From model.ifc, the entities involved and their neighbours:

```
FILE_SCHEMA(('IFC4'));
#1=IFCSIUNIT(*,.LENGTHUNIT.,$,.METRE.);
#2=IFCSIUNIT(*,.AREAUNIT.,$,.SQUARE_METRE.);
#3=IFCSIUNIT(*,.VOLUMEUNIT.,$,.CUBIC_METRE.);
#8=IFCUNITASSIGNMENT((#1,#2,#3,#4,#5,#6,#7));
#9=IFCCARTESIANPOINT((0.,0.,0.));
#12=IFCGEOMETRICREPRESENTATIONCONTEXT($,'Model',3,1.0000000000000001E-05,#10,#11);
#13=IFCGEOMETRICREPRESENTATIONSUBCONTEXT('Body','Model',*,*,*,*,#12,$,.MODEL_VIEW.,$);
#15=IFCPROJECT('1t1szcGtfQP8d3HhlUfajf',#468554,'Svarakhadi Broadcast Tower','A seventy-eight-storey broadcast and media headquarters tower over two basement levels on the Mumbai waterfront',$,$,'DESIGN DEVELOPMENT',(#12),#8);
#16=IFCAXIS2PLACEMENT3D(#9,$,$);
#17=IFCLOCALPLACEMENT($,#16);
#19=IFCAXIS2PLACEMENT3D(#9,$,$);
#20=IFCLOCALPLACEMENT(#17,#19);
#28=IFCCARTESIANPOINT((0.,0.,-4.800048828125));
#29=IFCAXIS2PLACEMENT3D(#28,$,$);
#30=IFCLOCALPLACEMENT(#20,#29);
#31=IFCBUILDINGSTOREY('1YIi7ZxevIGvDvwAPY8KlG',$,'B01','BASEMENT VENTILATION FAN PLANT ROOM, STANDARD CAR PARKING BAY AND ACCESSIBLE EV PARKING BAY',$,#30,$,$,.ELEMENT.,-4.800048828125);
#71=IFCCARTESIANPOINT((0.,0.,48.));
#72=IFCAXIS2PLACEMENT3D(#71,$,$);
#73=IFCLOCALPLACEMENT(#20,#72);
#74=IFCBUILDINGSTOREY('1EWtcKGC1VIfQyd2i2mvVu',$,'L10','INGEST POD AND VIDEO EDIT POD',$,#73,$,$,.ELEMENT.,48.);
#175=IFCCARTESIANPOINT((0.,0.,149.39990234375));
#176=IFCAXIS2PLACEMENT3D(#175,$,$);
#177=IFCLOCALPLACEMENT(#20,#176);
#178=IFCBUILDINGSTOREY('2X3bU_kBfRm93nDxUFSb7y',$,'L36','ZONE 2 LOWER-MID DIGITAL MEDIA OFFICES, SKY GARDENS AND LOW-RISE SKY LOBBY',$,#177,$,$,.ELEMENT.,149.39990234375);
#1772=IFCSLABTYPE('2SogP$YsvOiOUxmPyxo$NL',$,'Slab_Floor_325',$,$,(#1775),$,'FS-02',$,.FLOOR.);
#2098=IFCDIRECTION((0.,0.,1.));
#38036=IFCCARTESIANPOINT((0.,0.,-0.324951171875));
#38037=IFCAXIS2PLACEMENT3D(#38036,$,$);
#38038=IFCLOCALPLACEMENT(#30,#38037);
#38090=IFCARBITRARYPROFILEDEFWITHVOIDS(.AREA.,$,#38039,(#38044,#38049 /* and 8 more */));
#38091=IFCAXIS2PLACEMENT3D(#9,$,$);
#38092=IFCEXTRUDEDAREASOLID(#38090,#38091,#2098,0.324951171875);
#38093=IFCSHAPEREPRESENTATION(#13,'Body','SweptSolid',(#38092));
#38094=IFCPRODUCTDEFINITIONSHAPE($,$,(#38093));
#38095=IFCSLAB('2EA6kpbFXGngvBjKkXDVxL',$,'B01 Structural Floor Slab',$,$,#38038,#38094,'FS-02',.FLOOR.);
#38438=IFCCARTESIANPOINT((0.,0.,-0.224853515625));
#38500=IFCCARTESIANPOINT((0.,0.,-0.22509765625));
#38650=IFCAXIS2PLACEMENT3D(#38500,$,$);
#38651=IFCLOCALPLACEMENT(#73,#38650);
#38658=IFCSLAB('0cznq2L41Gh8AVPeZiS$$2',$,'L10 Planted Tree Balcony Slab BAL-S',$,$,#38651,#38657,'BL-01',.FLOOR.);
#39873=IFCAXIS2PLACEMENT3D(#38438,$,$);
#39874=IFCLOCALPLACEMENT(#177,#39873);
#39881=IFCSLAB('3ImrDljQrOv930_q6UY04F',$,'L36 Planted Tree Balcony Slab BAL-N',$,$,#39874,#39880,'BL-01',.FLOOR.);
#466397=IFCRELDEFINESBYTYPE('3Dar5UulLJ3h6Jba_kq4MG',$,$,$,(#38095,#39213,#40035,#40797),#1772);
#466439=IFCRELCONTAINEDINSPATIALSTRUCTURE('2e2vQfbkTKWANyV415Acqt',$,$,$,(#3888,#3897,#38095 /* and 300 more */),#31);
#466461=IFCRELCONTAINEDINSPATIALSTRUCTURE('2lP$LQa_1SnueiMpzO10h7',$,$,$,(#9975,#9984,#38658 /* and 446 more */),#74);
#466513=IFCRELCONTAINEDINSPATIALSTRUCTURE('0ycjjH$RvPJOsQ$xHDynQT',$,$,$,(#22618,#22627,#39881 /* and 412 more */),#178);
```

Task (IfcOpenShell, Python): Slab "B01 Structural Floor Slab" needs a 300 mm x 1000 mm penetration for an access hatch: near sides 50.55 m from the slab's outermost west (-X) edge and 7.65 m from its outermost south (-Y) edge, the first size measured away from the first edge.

```python
import numpy as np
import ifcopenshell
import ifcopenshell.api.feature
import ifcopenshell.api.geometry
import ifcopenshell.api.root
import ifcopenshell.geom
import ifcopenshell.util.placement
import ifcopenshell.util.representation
import ifcopenshell.util.shape
import ifcopenshell.util.unit

model = ifcopenshell.open("model.ifc")
unit_scale = ifcopenshell.util.unit.calculate_unit_scale(model)
settings = ifcopenshell.geom.settings()


def volume(element):
    """Net volume in cubic metres, openings subtracted."""
    shape = ifcopenshell.geom.create_shape(settings, element)
    return ifcopenshell.util.shape.get_volume(shape.geometry)


slab = model.by_guid("2EA6kpbFXGngvBjKkXDVxL")
before = volume(slab)

# Extent in the slab's own axes, in metres. The edges named are its -X and -Y sides.
slab_shape = ifcopenshell.geom.create_shape(settings, slab)
vertices = ifcopenshell.util.shape.get_vertices(slab_shape.geometry)
x_min, y_min, bottom = vertices.min(axis=0)
top = vertices[:, 2].max()

opening = ifcopenshell.api.root.create_entity(model, ifc_class="IfcOpeningElement", name="Access hatch opening", predefined_type="OPENING")
context = ifcopenshell.util.representation.get_context(model, "Model", "Body", "MODEL_VIEW")
width, depth = 0.3, 1
outline = [(0.0, 0.0), (width, 0.0), (width, depth), (0.0, depth), (0.0, 0.0)]
# Overshoot both faces by 50 mm so the cut is clean.
shape = ifcopenshell.api.geometry.add_slab_representation(
    model, context=context, depth=top - bottom + 0.1, polyline=outline
)
ifcopenshell.api.geometry.assign_representation(model, product=opening, representation=shape)

matrix = ifcopenshell.util.placement.get_local_placement(slab.ObjectPlacement)
matrix[:, 3] = matrix @ np.append(np.array([x_min + 50.55, y_min + 7.65, bottom - 0.05]) / unit_scale, 1.0)
ifcopenshell.api.geometry.edit_object_placement(model, product=opening, matrix=matrix, is_si=False)
ifcopenshell.api.feature.add_feature(model, feature=opening, element=slab)

after = volume(slab)

print(f"slab volume {before:.3f} -> {after:.3f} m3")

model.write("model_rev.ifc")
```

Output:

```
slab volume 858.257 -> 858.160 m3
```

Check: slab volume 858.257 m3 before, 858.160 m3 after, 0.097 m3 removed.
